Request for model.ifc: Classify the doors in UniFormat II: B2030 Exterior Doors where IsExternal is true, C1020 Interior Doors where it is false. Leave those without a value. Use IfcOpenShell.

First a look at what the model holds.

```python
import ifcopenshell
import ifcopenshell.util.element

model = ifcopenshell.open("model.ifc")
print(model.schema)
print("classifications:", [c.Name for c in model.by_type("IfcClassification")])
values = [ifcopenshell.util.element.get_pset(e, "Pset_DoorCommon", "IsExternal") for e in model.by_type("IfcDoor")]
for value in (True, False, None):
    print("IsExternal", value, values.count(value))
```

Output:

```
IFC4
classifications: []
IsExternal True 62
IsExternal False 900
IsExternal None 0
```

```python
import ifcopenshell
import ifcopenshell.api.classification
import ifcopenshell.util.element

model = ifcopenshell.open("model.ifc")

system = ifcopenshell.api.classification.add_classification(model, classification="UniFormat II")

doors = model.by_type("IfcDoor")
external = {e: ifcopenshell.util.element.get_pset(e, "Pset_DoorCommon", "IsExternal") for e in doors}
for flag, code, name in ((True, "B2030", "Exterior Doors"), (False, "C1020", "Interior Doors")):
    products = [e for e in doors if external[e] is flag]
    ifcopenshell.api.classification.add_reference(
        model, products=products, classification=system, identification=code, name=name
    )
    print(code, len(products))

model.write("model_edited.ifc")
```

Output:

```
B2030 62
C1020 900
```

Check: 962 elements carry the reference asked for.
